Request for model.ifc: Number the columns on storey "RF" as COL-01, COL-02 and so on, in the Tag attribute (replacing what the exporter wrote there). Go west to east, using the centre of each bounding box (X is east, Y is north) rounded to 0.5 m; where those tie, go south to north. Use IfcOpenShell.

First a look at what the model holds.

```python
import ifcopenshell
import ifcopenshell.util.element
import ifcopenshell.util.placement

model = ifcopenshell.open("model.ifc")
print(model.schema)
storey = next(s for s in model.by_type("IfcBuildingStorey") if s.Name == "RF")
columns = [e for e in ifcopenshell.util.element.get_decomposition(storey) if e.is_a("IfcColumn")]
for e in sorted(columns, key=lambda e: e.id()):
    origin = ifcopenshell.util.placement.get_local_placement(e.ObjectPlacement)[:3, 3]
    print(e.id(), e.Tag, e.Name, origin.round(2) + 0.0, sep=" | ")
```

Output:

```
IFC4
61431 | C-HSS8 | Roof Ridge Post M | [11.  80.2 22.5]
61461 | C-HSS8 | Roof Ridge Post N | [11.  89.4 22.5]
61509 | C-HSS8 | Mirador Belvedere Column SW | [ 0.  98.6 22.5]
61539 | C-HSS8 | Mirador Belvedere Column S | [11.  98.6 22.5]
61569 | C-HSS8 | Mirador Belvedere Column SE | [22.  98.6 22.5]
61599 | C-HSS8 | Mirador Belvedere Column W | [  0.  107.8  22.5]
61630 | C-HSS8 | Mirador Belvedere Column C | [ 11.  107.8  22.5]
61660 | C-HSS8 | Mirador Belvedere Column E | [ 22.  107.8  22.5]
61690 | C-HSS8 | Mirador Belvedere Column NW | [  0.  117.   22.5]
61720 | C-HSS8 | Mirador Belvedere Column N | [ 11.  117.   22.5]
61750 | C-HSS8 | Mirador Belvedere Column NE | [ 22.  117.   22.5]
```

```python
import ifcopenshell
import ifcopenshell.geom
import ifcopenshell.util.element
import ifcopenshell.util.shape

model = ifcopenshell.open("model.ifc")
settings = ifcopenshell.geom.settings()
settings.set("use-world-coords", True)


def centre(element):
    shape = ifcopenshell.geom.create_shape(settings, element)
    return ifcopenshell.util.shape.get_bbox_centroid(shape.geometry)


storey = next(s for s in model.by_type("IfcBuildingStorey") if s.Name == "RF")
columns = [e for e in ifcopenshell.util.element.get_decomposition(storey) if e.is_a("IfcColumn")]

# Insertion points can sit at a corner or the storey origin, so sort by the geometry (in metres).
centres = {e: centre(e) for e in columns}
columns.sort(key=lambda e: (round(centres[e][0] / 0.5), centres[e][1]))

for i, e in enumerate(columns, start=1):
    number = f"COL-{i:02d}"
    e.Tag = number
    print(e.id(), number)

model.write("model_v2.ifc")
```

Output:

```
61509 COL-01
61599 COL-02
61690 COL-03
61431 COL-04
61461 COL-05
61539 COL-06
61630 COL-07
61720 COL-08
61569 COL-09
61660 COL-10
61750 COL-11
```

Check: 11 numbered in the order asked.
